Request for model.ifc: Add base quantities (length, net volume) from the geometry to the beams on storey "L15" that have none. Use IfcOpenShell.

First a look at what the model holds.

```python
import ifcopenshell
import ifcopenshell.util.element
import ifcopenshell.util.unit

model = ifcopenshell.open("model.ifc")
print(model.schema)
for unit_type in ("LENGTHUNIT", "AREAUNIT", "VOLUMEUNIT"):
    print(unit_type, ifcopenshell.util.unit.calculate_unit_scale(model, unit_type))
storey = next(s for s in model.by_type("IfcBuildingStorey") if s.Name == "L15")
beams = [e for e in ifcopenshell.util.element.get_decomposition(storey) if e.is_a("IfcBeam")]
for e in sorted(beams, key=lambda e: e.id()):
    print(e.id(), e.is_a(), e.Name, list(ifcopenshell.util.element.get_psets(e, qtos_only=True)), sep=" | ")
```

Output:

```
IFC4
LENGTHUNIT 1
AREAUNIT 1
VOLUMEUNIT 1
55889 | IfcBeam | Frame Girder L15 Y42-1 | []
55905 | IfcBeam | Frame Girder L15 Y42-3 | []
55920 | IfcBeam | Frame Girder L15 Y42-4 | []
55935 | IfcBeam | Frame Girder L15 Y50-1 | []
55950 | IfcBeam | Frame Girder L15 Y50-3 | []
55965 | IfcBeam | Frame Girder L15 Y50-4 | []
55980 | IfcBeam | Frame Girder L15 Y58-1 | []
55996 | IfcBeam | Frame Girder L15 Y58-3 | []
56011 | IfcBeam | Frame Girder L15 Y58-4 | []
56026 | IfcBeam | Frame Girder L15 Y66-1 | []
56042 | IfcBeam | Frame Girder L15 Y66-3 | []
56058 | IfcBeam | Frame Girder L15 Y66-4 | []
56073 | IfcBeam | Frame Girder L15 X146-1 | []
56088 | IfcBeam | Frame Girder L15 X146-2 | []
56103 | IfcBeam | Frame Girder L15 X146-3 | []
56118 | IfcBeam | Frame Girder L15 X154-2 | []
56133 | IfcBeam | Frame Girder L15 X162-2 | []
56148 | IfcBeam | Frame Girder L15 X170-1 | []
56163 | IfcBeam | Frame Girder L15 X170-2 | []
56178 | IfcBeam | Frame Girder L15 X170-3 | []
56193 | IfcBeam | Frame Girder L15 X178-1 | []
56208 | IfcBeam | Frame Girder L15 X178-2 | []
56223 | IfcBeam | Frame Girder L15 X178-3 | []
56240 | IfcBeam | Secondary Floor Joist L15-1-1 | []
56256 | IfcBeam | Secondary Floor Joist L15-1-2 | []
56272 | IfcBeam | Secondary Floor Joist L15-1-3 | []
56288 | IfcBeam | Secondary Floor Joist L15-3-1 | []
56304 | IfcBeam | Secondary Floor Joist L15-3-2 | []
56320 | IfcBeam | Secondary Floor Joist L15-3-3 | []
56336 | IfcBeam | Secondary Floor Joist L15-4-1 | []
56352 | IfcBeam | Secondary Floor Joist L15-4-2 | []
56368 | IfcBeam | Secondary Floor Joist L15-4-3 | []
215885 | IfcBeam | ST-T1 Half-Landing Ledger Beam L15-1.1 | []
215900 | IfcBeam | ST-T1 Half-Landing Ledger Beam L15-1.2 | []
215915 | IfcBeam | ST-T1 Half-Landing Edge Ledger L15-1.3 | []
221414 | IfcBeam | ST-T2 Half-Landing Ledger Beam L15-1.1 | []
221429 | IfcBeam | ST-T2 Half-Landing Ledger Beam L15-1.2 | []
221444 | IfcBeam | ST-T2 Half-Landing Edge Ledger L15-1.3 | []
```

```python
import ifcopenshell
import ifcopenshell.api.pset
import ifcopenshell.geom
import ifcopenshell.util.element
import ifcopenshell.util.shape
import ifcopenshell.util.unit

model = ifcopenshell.open("model.ifc")
unit_scale = ifcopenshell.util.unit.calculate_unit_scale(model)
volume_scale = ifcopenshell.util.unit.calculate_unit_scale(model, "VOLUMEUNIT")
settings = ifcopenshell.geom.settings()

storey = next(s for s in model.by_type("IfcBuildingStorey") if s.Name == "L15")
beams = [e for e in ifcopenshell.util.element.get_decomposition(storey) if e.is_a("IfcBeam")]

for e in sorted(beams, key=lambda e: e.id()):
    if ifcopenshell.util.element.get_psets(e, qtos_only=True, should_inherit=False):
        continue
    # Geometry comes back in metres, in the element's own axes.
    shape = ifcopenshell.geom.create_shape(settings, e)
    values = {
        "Length": ifcopenshell.util.shape.get_max_xyz(shape.geometry) / unit_scale,
        "NetVolume": ifcopenshell.util.shape.get_volume(shape.geometry) / volume_scale,
    }
    qto = ifcopenshell.api.pset.add_qto(model, product=e, name="Qto_BeamBaseQuantities")
    ifcopenshell.api.pset.edit_qto(model, qto=qto, properties=values)
    print(e.id(), {k: round(v, 3) for k, v in values.items()})

model.write("model_updated.ifc")
```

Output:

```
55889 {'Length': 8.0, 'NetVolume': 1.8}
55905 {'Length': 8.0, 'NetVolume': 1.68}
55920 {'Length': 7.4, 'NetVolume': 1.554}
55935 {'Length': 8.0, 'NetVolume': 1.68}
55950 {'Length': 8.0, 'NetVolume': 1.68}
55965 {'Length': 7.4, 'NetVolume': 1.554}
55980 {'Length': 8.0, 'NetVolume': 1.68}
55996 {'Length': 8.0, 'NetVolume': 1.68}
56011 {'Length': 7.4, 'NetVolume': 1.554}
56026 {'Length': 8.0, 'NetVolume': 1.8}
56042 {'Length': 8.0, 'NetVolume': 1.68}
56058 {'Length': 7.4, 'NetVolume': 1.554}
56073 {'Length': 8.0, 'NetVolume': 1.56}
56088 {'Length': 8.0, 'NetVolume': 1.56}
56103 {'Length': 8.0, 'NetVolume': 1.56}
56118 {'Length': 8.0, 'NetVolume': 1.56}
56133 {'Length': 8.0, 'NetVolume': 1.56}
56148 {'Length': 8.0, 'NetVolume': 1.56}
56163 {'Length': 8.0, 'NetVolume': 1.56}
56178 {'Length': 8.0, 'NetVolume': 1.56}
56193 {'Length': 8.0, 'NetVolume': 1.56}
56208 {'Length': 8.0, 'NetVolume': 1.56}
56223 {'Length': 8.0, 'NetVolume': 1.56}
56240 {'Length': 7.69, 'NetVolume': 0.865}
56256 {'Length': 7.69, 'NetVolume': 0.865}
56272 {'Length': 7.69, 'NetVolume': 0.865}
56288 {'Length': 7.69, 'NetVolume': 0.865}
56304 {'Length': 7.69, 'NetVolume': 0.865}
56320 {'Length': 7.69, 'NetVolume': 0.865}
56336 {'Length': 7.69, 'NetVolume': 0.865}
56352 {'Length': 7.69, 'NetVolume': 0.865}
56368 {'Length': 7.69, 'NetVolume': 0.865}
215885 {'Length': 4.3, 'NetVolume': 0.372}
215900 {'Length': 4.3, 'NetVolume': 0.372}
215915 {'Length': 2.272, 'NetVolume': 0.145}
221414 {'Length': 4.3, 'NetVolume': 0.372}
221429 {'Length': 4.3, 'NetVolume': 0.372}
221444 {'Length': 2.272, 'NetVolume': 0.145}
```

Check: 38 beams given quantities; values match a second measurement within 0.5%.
